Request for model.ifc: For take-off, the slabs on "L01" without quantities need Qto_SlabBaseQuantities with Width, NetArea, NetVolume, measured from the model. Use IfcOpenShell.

First a look at what the model holds.

```python
import ifcopenshell
import ifcopenshell.util.element
import ifcopenshell.util.unit

model = ifcopenshell.open("model.ifc")
print(model.schema)
for unit_type in ("LENGTHUNIT", "AREAUNIT", "VOLUMEUNIT"):
    print(unit_type, ifcopenshell.util.unit.calculate_unit_scale(model, unit_type))
storey = next(s for s in model.by_type("IfcBuildingStorey") if s.Name == "L01")
slabs = [e for e in ifcopenshell.util.element.get_decomposition(storey) if e.is_a("IfcSlab")]
for e in sorted(slabs, key=lambda e: e.id()):
    print(e.id(), e.is_a(), e.Name, list(ifcopenshell.util.element.get_psets(e, qtos_only=True)), sep=" | ")
```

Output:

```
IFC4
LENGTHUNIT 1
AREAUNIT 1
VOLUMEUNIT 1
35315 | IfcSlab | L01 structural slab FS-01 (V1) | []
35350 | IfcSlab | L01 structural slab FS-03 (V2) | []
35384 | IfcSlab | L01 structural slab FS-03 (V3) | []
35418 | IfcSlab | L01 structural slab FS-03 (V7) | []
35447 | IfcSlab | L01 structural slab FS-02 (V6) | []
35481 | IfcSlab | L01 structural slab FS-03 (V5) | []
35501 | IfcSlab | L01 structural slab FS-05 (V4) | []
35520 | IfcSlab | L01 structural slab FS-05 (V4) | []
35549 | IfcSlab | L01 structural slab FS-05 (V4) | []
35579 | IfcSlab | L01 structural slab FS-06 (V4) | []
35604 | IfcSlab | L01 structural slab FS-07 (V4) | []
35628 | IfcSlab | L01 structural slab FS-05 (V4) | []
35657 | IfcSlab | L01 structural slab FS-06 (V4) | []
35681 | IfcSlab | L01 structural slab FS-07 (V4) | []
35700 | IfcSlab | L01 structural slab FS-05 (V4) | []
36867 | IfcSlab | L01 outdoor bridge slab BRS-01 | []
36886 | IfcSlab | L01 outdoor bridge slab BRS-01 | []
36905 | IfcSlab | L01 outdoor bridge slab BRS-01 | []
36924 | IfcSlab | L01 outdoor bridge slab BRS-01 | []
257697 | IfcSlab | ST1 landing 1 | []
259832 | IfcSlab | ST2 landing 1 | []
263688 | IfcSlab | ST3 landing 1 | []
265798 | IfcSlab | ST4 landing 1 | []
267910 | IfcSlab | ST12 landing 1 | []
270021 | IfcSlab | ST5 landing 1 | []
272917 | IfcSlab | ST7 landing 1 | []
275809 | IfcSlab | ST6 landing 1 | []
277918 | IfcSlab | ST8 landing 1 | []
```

```python
import ifcopenshell
import ifcopenshell.api.pset
import ifcopenshell.geom
import ifcopenshell.util.element
import ifcopenshell.util.shape
import ifcopenshell.util.unit

model = ifcopenshell.open("model.ifc")
unit_scale = ifcopenshell.util.unit.calculate_unit_scale(model)
area_scale = ifcopenshell.util.unit.calculate_unit_scale(model, "AREAUNIT")
volume_scale = ifcopenshell.util.unit.calculate_unit_scale(model, "VOLUMEUNIT")
settings = ifcopenshell.geom.settings()

storey = next(s for s in model.by_type("IfcBuildingStorey") if s.Name == "L01")
slabs = [e for e in ifcopenshell.util.element.get_decomposition(storey) if e.is_a("IfcSlab")]

for e in sorted(slabs, key=lambda e: e.id()):
    if ifcopenshell.util.element.get_psets(e, qtos_only=True, should_inherit=False):
        continue
    # Geometry comes back in metres, in the element's own axes.
    shape = ifcopenshell.geom.create_shape(settings, e)
    values = {
        "Width": ifcopenshell.util.shape.get_z(shape.geometry) / unit_scale,
        "NetArea": ifcopenshell.util.shape.get_footprint_area(shape.geometry) / area_scale,
        "NetVolume": ifcopenshell.util.shape.get_volume(shape.geometry) / volume_scale,
    }
    qto = ifcopenshell.api.pset.add_qto(model, product=e, name="Qto_SlabBaseQuantities")
    ifcopenshell.api.pset.edit_qto(model, qto=qto, properties=values)
    print(e.id(), {k: round(v, 3) for k, v in values.items()})

model.write("model_v2.ifc")
```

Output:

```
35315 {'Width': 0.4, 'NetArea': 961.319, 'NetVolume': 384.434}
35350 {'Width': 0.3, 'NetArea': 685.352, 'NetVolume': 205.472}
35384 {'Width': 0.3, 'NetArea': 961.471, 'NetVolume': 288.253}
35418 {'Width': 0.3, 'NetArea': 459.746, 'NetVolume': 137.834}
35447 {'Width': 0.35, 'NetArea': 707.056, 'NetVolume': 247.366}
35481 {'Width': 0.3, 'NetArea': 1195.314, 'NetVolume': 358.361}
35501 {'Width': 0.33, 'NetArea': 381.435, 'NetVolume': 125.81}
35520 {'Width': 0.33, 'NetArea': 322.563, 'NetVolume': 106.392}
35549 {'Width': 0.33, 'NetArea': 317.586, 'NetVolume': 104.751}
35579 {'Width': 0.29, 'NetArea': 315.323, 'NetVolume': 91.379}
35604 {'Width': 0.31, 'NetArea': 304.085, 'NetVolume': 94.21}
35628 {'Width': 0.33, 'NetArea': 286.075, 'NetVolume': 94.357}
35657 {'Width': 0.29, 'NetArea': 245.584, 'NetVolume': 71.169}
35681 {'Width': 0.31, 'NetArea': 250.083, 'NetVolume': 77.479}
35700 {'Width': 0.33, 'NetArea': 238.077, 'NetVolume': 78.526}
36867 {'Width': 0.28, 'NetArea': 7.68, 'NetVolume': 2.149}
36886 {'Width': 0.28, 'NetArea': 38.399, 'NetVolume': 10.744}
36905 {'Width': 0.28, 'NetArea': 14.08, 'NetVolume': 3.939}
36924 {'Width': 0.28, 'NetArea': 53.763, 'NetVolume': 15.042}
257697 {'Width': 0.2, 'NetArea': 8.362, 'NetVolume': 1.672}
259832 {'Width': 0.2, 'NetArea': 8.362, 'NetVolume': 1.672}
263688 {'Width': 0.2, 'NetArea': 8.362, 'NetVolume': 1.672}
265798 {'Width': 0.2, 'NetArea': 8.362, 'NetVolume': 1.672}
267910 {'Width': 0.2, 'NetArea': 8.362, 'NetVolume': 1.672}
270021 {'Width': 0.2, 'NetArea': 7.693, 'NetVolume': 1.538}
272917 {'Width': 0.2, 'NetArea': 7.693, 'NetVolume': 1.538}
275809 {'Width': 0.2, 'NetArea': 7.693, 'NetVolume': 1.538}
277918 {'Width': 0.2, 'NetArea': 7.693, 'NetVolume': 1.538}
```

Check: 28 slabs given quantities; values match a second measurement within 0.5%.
